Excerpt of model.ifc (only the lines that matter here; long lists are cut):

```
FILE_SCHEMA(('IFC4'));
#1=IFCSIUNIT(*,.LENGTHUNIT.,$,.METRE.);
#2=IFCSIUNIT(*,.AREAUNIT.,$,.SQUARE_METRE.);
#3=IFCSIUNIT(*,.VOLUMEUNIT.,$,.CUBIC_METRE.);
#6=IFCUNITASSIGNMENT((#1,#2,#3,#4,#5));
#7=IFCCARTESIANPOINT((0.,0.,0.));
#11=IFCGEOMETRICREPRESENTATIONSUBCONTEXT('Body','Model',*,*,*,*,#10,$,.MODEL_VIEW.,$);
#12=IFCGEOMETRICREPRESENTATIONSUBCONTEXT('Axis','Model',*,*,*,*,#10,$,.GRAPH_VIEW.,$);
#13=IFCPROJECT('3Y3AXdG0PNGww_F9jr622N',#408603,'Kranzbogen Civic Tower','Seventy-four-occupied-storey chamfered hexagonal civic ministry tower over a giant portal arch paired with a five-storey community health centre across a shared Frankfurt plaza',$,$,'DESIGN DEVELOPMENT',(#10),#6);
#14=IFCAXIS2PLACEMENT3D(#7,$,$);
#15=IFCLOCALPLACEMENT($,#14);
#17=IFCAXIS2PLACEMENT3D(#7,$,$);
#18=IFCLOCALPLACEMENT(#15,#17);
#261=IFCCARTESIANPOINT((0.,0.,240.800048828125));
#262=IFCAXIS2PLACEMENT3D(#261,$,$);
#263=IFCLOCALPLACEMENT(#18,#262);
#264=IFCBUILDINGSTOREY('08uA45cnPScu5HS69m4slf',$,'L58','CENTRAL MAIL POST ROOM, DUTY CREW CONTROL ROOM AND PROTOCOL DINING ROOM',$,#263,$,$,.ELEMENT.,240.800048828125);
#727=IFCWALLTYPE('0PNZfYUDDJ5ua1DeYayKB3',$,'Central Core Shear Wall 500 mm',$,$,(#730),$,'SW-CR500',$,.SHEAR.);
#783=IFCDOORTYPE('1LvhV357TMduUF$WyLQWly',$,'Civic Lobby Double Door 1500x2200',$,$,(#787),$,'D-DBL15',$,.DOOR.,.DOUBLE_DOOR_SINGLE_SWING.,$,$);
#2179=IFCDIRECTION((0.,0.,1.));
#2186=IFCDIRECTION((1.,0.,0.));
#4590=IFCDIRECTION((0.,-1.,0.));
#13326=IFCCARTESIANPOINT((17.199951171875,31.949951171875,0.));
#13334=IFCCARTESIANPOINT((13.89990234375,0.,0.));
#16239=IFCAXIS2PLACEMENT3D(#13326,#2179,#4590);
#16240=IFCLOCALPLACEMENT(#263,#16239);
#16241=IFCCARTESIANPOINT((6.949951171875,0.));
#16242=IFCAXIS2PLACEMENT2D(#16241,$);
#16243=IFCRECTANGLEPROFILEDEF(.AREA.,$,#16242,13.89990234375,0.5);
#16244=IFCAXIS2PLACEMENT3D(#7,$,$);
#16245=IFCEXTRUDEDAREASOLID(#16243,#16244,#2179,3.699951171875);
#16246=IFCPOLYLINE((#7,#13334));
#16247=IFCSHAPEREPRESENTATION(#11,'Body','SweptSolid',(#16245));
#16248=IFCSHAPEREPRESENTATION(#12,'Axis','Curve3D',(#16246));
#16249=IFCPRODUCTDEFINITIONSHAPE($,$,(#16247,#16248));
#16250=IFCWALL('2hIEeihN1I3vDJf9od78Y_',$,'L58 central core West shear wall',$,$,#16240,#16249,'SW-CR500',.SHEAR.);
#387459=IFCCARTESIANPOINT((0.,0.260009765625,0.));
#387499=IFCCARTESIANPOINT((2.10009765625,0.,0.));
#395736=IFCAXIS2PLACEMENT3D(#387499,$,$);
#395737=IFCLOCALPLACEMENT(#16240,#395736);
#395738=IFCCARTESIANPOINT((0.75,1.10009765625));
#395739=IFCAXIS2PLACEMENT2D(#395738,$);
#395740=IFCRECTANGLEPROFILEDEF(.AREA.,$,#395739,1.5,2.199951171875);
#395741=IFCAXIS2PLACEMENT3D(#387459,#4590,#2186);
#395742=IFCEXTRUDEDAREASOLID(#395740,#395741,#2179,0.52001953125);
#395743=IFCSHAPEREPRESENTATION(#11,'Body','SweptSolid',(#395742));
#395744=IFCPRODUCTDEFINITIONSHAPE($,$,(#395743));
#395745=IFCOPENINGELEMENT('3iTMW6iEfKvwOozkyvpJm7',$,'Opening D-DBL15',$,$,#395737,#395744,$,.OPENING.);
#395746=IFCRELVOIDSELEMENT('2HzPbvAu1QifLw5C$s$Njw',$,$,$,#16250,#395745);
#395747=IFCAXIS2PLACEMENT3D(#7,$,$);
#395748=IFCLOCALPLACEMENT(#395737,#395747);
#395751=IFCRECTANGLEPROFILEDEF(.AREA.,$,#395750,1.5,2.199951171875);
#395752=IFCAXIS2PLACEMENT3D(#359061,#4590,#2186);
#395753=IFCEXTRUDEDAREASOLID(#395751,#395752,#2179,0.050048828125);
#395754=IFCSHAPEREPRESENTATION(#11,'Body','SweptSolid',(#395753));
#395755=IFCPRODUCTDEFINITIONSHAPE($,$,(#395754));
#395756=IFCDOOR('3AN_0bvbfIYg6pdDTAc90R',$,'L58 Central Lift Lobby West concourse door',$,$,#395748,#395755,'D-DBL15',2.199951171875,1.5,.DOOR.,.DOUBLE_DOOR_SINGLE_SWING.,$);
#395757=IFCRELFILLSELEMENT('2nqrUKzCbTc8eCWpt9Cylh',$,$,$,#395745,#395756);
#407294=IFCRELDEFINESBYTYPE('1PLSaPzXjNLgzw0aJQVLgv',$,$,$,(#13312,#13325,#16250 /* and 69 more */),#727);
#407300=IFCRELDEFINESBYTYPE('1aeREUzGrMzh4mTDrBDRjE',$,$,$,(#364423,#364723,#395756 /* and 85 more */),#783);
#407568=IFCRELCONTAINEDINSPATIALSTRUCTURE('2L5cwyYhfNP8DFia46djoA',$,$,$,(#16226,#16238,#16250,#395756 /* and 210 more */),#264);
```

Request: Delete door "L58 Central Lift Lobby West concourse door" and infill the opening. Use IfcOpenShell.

```python
import ifcopenshell
import ifcopenshell.api.feature
import ifcopenshell.api.root
import ifcopenshell.geom
import ifcopenshell.util.shape

model = ifcopenshell.open("model.ifc")
settings = ifcopenshell.geom.settings()


def volume(element):
    """Net volume in cubic metres, openings subtracted."""
    shape = ifcopenshell.geom.create_shape(settings, element)
    return ifcopenshell.util.shape.get_volume(shape.geometry)


door = model.by_guid("3AN_0bvbfIYg6pdDTAc90R")
opening = door.FillsVoids[0].RelatingOpeningElement
wall = opening.VoidsElements[0].RelatingBuildingElement
before = volume(wall)

ifcopenshell.api.root.remove_product(model, product=door)
ifcopenshell.api.feature.remove_feature(model, feature=opening)

after = volume(wall)

print(f"wall volume {before:.3f} -> {after:.3f} m3")

model.write("model-out.ifc")
```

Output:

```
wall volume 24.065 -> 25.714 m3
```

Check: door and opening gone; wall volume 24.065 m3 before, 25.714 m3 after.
